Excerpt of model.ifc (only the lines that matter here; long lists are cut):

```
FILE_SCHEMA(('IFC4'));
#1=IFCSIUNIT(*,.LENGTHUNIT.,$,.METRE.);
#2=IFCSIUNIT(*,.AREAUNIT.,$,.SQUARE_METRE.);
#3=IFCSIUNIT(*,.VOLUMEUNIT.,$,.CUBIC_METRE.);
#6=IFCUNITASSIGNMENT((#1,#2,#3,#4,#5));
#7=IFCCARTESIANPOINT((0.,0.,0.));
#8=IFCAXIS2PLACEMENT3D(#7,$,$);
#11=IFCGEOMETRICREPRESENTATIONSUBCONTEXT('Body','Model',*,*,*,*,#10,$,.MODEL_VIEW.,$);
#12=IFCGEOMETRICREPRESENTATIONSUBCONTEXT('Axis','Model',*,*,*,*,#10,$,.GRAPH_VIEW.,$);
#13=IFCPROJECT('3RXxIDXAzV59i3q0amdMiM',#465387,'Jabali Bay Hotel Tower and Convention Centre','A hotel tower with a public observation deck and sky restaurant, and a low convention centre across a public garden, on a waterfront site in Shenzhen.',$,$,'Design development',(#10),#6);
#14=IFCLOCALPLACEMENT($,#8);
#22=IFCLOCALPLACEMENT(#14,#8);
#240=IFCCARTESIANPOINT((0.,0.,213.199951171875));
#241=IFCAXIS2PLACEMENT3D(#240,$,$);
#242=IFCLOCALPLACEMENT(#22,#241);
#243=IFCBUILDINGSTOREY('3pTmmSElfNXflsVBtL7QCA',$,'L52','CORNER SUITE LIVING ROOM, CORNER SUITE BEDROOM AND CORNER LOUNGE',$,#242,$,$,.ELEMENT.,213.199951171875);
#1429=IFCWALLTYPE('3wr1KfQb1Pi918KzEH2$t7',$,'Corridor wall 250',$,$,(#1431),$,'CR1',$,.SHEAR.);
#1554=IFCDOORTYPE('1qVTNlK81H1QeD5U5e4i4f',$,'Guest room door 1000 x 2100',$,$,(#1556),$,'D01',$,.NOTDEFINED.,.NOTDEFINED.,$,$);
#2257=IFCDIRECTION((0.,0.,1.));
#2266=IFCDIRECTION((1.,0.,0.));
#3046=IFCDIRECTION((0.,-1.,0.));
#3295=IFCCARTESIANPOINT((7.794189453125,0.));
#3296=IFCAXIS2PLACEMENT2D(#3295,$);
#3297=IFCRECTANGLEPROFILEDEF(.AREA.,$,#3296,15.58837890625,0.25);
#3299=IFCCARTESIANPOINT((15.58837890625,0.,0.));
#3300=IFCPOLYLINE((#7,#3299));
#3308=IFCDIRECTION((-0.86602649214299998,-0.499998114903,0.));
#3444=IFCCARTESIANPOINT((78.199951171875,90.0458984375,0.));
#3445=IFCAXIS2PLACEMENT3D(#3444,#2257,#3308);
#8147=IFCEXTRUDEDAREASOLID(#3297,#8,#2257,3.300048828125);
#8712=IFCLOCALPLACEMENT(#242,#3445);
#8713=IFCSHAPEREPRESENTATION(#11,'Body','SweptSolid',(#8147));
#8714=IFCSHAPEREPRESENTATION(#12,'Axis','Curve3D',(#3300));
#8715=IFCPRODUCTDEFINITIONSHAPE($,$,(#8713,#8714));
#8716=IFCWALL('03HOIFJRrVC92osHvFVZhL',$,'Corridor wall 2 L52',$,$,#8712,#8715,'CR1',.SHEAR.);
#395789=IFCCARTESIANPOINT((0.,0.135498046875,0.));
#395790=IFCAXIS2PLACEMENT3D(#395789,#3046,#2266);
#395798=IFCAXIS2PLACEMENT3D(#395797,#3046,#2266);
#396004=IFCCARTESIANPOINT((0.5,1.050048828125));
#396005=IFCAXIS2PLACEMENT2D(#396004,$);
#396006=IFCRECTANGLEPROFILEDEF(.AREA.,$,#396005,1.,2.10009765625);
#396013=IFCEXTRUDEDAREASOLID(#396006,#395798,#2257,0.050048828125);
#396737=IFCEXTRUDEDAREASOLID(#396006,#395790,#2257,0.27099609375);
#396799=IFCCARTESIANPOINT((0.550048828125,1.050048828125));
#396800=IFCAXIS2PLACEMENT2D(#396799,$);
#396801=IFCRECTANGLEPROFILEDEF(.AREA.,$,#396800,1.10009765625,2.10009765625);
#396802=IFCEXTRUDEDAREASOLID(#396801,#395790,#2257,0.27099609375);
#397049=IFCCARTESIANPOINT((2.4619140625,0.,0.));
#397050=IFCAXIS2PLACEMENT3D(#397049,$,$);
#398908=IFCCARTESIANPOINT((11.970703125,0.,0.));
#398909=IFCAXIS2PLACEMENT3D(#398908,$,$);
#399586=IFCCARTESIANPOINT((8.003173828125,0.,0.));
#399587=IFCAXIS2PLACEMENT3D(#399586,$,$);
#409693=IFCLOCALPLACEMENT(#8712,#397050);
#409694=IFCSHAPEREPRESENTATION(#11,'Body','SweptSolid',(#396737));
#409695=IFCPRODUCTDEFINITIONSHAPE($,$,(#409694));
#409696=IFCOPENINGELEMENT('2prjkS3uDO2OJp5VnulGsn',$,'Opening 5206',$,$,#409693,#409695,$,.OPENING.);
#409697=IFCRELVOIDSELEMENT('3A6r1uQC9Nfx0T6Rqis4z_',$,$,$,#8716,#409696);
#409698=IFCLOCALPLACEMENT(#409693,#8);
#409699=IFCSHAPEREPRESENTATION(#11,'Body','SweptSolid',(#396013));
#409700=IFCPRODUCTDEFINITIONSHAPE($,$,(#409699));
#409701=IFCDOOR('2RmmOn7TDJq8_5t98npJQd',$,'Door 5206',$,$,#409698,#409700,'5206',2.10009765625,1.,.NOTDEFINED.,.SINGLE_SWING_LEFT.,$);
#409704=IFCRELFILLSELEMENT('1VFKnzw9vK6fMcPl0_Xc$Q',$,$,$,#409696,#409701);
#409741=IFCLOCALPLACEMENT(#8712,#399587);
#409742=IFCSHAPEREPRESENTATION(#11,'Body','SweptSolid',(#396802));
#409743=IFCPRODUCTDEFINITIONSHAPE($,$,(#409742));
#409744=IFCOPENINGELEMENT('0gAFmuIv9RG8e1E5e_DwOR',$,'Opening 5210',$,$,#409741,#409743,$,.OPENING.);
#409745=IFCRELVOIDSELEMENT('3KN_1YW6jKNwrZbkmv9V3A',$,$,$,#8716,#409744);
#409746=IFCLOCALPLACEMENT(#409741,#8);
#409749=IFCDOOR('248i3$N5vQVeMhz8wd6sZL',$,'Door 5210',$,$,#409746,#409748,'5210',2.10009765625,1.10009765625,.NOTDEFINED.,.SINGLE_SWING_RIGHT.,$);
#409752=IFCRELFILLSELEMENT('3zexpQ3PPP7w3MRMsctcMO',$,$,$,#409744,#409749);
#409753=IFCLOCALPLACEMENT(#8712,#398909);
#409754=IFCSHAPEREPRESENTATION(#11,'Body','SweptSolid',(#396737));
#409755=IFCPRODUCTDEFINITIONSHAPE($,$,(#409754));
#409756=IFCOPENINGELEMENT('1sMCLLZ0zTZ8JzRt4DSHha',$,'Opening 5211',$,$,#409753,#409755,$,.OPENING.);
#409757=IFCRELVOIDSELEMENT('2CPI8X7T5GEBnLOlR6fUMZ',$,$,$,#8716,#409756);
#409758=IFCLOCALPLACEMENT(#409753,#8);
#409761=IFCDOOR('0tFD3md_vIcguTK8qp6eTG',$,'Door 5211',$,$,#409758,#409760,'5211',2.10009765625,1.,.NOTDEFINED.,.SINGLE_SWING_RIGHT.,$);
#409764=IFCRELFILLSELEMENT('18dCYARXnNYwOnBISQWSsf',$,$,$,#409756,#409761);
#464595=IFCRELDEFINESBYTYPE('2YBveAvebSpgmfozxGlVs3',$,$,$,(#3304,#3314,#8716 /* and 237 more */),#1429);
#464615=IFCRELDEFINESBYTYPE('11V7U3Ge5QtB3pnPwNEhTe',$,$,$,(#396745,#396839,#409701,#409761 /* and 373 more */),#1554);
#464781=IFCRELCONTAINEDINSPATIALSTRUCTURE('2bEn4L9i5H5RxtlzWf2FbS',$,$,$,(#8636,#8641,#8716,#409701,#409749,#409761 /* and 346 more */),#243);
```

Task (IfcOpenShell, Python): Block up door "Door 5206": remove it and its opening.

```python
import ifcopenshell
import ifcopenshell.api.feature
import ifcopenshell.api.root
import ifcopenshell.geom
import ifcopenshell.util.shape

model = ifcopenshell.open("model.ifc")
settings = ifcopenshell.geom.settings()


def volume(element):
    """Net volume in cubic metres, openings subtracted."""
    shape = ifcopenshell.geom.create_shape(settings, element)
    return ifcopenshell.util.shape.get_volume(shape.geometry)


door = model.by_guid("2RmmOn7TDJq8_5t98npJQd")
opening = door.FillsVoids[0].RelatingOpeningElement
wall = opening.VoidsElements[0].RelatingBuildingElement
before = volume(wall)

ifcopenshell.api.root.remove_product(model, product=door)
ifcopenshell.api.feature.remove_feature(model, feature=opening)

after = volume(wall)

print(f"wall volume {before:.3f} -> {after:.3f} m3")

model.write("model_updated.ifc")
```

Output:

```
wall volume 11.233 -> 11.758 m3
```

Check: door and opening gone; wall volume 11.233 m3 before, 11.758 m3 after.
